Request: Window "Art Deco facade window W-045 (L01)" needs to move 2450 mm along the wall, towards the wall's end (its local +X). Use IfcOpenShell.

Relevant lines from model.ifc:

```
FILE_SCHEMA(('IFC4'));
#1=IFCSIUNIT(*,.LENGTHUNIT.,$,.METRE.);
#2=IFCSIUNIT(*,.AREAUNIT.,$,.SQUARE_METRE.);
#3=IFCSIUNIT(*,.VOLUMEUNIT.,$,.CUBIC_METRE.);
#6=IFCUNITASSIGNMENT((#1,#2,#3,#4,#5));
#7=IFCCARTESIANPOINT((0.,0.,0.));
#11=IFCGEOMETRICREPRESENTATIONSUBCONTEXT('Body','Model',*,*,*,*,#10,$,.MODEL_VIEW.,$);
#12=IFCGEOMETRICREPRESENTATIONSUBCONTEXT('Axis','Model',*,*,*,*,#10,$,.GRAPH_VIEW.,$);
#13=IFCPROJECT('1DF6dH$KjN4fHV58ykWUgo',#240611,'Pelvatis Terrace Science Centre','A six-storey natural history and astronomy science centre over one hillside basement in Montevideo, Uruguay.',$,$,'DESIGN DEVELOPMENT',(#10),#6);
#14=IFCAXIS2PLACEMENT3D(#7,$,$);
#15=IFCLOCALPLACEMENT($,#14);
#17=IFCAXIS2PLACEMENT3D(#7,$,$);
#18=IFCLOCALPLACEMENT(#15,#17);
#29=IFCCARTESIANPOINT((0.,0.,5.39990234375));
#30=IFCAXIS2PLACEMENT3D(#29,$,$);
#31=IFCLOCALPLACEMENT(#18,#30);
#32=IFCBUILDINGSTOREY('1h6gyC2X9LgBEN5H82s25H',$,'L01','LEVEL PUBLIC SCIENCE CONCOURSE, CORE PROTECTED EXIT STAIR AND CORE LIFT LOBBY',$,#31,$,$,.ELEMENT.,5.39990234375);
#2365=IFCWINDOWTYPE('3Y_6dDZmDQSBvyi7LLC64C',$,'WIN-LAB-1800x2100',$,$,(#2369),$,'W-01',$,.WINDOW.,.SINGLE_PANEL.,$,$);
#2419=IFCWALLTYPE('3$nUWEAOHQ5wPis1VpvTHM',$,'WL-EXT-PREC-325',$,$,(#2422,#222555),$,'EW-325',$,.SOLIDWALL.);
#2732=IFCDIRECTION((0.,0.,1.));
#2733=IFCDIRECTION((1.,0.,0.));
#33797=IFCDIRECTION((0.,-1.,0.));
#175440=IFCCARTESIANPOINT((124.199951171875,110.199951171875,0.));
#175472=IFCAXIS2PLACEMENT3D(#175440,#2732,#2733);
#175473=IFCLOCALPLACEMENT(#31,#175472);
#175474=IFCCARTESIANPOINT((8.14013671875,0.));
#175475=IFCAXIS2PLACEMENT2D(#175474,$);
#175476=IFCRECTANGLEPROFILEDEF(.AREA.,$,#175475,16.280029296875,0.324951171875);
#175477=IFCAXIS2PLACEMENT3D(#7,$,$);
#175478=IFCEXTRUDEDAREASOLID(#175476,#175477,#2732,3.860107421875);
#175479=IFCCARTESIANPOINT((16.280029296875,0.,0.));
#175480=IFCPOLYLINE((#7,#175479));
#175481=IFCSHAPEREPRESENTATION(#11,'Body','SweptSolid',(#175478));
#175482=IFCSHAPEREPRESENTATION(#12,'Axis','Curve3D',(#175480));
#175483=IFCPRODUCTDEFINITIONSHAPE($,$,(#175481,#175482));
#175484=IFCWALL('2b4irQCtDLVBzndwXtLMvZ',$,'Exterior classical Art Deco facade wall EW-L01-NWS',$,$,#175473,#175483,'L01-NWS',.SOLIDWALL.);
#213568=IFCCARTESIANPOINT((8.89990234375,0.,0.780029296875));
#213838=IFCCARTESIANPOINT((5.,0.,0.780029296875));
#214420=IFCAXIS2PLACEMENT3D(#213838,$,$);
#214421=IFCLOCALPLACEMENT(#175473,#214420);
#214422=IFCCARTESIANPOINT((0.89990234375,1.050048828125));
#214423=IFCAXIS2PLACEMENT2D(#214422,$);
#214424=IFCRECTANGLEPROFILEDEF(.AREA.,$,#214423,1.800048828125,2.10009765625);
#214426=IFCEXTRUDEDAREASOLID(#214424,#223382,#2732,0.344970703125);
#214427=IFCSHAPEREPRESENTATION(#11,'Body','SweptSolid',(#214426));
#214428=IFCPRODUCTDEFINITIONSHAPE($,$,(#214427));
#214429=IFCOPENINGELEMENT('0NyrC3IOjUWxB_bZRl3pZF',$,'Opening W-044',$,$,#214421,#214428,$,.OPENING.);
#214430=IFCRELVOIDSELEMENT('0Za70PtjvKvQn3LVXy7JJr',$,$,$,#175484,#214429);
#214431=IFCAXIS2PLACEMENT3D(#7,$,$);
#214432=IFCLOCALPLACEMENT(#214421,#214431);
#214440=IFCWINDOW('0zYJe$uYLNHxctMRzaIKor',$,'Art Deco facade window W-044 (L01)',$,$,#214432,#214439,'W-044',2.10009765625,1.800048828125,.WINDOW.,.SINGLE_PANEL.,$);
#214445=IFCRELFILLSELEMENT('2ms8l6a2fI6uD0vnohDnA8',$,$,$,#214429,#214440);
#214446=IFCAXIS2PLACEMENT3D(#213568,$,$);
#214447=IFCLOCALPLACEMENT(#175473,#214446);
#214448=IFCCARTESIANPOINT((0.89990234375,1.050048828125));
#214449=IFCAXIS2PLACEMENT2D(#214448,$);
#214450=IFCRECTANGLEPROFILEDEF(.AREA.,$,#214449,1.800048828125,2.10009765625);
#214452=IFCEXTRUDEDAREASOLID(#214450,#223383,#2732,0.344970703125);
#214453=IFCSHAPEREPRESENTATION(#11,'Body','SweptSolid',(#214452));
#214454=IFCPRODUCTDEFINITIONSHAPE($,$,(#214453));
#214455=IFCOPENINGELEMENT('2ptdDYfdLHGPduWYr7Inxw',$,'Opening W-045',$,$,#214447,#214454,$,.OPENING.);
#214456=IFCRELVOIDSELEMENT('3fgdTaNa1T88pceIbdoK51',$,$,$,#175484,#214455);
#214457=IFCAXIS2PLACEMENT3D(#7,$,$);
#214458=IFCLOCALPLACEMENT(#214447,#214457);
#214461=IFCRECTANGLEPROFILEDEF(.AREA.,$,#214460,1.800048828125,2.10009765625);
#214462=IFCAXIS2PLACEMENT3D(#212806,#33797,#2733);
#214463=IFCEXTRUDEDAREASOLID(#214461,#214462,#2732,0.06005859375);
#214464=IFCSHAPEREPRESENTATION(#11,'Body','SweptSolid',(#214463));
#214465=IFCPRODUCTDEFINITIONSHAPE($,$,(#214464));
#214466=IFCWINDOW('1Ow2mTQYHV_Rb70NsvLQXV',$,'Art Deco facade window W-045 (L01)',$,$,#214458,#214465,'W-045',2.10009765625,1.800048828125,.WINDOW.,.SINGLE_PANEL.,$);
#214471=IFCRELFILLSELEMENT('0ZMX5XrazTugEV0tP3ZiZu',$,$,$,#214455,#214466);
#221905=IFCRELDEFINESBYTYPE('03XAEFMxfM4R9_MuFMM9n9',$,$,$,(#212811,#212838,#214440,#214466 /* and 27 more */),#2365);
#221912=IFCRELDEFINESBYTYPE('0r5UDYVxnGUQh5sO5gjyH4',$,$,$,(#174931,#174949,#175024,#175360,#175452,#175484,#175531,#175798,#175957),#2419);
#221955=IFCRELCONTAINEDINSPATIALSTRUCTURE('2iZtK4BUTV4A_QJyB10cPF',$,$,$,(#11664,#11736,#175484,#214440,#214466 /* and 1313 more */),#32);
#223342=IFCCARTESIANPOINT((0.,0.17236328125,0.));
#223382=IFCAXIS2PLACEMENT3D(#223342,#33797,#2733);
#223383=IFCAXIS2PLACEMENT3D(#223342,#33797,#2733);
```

```python
import ifcopenshell
import ifcopenshell.api.geometry
import ifcopenshell.util.placement

model = ifcopenshell.open("model.ifc")

window = model.by_guid("1Ow2mTQYHV_Rb70NsvLQXV")
opening = window.FillsVoids[0].RelatingOpeningElement
wall = opening.VoidsElements[0].RelatingBuildingElement

wall_matrix = ifcopenshell.util.placement.get_local_placement(wall.ObjectPlacement)
shift = wall_matrix[:3, 0] * 2.45
before = ifcopenshell.util.placement.get_local_placement(window.ObjectPlacement)[:3, 3].copy()

# The window is placed relative to its opening, so it follows when the opening moves.
matrix = ifcopenshell.util.placement.get_local_placement(opening.ObjectPlacement)
matrix[:3, 3] += shift
ifcopenshell.api.geometry.edit_object_placement(
    model, product=opening, matrix=matrix, is_si=False, should_transform_children=True
)

after = ifcopenshell.util.placement.get_local_placement(window.ObjectPlacement)[:3, 3]
print("window moved by", (after - before).round(3) + 0.0)

model.write("model_updated.ifc")
```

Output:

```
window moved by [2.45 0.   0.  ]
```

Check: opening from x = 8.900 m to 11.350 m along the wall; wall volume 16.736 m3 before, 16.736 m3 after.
